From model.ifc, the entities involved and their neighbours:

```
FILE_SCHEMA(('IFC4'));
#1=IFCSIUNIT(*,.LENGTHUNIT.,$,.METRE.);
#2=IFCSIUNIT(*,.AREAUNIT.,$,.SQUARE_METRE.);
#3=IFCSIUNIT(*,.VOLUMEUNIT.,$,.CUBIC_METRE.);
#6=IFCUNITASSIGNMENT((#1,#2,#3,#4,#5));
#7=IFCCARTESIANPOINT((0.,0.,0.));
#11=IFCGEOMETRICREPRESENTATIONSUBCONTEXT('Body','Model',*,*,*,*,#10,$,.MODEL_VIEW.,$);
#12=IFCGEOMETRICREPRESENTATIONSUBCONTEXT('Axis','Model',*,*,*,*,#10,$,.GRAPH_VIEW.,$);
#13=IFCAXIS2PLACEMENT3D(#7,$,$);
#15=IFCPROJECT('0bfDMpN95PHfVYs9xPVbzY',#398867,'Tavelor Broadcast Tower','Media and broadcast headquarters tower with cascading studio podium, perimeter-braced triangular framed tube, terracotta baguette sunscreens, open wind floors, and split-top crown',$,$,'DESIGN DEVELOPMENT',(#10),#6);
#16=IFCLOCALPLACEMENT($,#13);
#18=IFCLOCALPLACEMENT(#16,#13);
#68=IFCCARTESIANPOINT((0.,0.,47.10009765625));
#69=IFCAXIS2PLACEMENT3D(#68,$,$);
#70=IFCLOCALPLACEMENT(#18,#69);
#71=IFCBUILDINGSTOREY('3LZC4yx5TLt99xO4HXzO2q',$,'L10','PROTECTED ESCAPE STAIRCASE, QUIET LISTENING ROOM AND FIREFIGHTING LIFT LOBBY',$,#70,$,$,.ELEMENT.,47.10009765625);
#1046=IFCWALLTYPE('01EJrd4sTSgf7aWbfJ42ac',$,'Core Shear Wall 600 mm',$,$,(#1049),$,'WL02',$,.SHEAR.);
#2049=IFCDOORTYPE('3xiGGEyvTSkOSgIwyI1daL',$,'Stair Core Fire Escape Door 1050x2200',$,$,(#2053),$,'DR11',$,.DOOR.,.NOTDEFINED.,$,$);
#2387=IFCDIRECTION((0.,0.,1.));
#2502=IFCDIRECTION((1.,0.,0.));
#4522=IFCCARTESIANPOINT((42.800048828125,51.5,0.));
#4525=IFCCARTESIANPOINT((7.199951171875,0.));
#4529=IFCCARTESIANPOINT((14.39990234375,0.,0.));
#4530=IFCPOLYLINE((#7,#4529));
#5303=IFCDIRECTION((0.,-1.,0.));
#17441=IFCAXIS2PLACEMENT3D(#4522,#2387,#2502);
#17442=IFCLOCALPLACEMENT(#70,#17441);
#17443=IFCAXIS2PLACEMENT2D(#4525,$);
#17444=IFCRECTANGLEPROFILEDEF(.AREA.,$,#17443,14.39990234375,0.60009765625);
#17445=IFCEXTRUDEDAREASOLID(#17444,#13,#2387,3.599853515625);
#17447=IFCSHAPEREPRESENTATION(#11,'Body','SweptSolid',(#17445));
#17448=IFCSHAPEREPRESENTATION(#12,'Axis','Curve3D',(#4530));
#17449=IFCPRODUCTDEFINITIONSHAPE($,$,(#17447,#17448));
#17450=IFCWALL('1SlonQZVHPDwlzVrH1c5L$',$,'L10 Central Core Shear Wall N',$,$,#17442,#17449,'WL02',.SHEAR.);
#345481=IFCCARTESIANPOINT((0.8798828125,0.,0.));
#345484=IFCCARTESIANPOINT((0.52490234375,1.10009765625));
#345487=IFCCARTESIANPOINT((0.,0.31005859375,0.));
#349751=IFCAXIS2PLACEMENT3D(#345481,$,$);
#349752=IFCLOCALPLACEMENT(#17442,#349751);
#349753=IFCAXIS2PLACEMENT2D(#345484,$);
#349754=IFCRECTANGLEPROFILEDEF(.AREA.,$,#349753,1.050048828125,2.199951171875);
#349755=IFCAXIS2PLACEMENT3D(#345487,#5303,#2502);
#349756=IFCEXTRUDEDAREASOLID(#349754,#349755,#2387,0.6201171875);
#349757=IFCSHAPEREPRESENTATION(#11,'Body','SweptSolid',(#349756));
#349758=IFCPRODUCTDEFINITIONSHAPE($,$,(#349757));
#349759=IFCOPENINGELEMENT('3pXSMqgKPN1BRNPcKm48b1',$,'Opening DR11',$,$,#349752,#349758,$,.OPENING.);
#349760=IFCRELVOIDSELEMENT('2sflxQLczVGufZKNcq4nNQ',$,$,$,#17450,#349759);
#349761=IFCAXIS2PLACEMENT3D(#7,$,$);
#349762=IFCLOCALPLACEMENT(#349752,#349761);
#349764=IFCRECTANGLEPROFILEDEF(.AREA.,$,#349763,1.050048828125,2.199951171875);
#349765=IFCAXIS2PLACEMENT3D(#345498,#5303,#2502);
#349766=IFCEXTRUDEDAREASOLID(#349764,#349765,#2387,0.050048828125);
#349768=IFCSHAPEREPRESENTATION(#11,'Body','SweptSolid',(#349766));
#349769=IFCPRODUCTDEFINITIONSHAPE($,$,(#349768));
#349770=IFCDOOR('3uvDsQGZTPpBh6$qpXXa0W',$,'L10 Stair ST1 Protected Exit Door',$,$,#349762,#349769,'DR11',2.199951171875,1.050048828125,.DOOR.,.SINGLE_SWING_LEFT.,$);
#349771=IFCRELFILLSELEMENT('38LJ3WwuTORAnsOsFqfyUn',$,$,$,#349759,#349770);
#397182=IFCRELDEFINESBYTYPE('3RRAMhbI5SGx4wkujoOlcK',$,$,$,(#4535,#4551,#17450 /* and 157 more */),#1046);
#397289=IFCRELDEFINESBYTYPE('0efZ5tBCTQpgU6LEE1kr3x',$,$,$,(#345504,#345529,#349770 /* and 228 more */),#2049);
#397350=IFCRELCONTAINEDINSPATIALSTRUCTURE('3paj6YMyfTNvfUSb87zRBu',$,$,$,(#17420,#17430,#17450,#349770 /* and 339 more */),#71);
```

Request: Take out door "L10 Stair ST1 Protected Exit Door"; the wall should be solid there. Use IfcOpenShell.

```python
import ifcopenshell
import ifcopenshell.api.feature
import ifcopenshell.api.root
import ifcopenshell.geom
import ifcopenshell.util.shape

model = ifcopenshell.open("model.ifc")
settings = ifcopenshell.geom.settings()


def volume(element):
    """Net volume in cubic metres, openings subtracted."""
    shape = ifcopenshell.geom.create_shape(settings, element)
    return ifcopenshell.util.shape.get_volume(shape.geometry)


door = model.by_id(349770)
opening = door.FillsVoids[0].RelatingOpeningElement
wall = opening.VoidsElements[0].RelatingBuildingElement
before = volume(wall)

ifcopenshell.api.root.remove_product(model, product=door)
ifcopenshell.api.feature.remove_feature(model, feature=opening)

after = volume(wall)

print(f"wall volume {before:.3f} -> {after:.3f} m3")

model.write("model_edited.ifc")
```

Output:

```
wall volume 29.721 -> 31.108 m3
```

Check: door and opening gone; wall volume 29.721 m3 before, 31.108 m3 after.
